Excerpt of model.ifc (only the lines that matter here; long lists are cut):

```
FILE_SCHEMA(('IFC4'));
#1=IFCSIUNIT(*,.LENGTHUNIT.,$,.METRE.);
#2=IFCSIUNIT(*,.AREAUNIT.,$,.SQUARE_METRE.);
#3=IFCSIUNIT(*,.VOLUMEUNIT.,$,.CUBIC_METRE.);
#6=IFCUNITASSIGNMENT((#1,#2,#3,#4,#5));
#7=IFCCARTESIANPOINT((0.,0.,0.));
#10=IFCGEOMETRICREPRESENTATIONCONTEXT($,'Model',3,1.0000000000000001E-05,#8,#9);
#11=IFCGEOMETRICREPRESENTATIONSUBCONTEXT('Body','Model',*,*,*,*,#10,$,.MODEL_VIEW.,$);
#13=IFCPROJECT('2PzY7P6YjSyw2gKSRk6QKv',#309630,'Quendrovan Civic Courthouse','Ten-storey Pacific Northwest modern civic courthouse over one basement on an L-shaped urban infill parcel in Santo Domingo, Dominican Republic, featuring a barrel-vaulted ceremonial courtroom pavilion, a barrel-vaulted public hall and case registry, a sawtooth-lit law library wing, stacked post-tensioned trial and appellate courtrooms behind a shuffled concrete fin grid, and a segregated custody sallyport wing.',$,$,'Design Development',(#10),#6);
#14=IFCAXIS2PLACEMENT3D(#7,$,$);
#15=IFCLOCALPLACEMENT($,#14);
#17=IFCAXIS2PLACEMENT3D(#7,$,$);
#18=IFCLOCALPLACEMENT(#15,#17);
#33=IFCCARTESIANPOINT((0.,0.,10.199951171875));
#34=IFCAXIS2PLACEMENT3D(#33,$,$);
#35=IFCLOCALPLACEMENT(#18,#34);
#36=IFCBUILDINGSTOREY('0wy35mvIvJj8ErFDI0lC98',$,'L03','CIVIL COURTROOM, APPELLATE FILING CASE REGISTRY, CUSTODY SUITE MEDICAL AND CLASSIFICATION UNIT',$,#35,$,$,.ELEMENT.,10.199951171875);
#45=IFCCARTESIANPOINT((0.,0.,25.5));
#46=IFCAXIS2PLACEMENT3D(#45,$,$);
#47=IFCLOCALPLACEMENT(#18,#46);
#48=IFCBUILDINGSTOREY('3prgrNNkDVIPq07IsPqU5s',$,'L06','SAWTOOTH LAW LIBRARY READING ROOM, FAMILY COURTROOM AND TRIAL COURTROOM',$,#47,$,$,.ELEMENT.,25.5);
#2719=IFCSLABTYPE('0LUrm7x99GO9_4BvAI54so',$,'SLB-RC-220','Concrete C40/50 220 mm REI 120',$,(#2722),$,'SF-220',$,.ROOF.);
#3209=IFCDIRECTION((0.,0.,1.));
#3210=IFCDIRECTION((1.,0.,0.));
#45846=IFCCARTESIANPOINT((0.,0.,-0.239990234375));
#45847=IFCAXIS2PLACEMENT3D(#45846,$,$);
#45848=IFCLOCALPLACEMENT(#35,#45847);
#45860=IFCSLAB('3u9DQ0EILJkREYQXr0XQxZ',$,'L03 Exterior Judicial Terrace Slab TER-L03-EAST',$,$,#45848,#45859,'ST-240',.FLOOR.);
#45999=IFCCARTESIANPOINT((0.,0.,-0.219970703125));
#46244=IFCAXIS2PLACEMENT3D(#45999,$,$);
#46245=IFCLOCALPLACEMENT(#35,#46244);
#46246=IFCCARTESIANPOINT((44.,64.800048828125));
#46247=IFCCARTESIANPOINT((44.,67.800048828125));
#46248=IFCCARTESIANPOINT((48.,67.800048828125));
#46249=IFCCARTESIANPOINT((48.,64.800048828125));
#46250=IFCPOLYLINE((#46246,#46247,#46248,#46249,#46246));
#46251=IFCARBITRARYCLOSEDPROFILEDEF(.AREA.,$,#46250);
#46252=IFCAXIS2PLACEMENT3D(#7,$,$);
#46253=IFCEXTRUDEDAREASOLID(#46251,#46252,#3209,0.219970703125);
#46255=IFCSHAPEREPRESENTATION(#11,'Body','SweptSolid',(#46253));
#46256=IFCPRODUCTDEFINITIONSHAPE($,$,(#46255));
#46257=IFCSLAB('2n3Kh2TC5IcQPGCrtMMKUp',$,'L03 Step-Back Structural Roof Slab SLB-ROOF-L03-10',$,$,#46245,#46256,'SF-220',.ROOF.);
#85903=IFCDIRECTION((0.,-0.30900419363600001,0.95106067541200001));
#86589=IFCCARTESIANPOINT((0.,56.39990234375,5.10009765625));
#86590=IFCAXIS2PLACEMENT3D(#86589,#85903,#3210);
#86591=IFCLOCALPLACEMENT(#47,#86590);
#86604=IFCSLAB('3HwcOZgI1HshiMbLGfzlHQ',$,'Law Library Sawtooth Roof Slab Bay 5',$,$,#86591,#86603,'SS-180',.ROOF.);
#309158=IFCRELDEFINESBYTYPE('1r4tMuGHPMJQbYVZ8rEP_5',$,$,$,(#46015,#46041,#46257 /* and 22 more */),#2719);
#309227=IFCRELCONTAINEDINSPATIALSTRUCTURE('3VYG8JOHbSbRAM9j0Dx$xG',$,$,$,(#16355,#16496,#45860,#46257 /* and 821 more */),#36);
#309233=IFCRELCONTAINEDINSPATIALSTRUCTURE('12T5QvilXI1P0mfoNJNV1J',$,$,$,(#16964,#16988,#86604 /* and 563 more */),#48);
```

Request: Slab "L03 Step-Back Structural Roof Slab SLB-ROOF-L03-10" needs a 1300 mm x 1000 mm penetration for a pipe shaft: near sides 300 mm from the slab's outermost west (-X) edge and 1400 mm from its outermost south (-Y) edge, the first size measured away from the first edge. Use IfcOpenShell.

```python
import numpy as np
import ifcopenshell
import ifcopenshell.api.feature
import ifcopenshell.api.geometry
import ifcopenshell.api.root
import ifcopenshell.geom
import ifcopenshell.util.placement
import ifcopenshell.util.representation
import ifcopenshell.util.shape
import ifcopenshell.util.unit

model = ifcopenshell.open("model.ifc")
unit_scale = ifcopenshell.util.unit.calculate_unit_scale(model)
settings = ifcopenshell.geom.settings()


def volume(element):
    """Net volume in cubic metres, openings subtracted."""
    shape = ifcopenshell.geom.create_shape(settings, element)
    return ifcopenshell.util.shape.get_volume(shape.geometry)


slab = model.by_guid("2n3Kh2TC5IcQPGCrtMMKUp")
before = volume(slab)

# Extent in the slab's own axes, in metres. The edges named are its -X and -Y sides.
slab_shape = ifcopenshell.geom.create_shape(settings, slab)
vertices = ifcopenshell.util.shape.get_vertices(slab_shape.geometry)
x_min, y_min, bottom = vertices.min(axis=0)
top = vertices[:, 2].max()

opening = ifcopenshell.api.root.create_entity(model, ifc_class="IfcOpeningElement", name="Pipe shaft opening", predefined_type="OPENING")
context = ifcopenshell.util.representation.get_context(model, "Model", "Body", "MODEL_VIEW")
width, depth = 1.3, 1
outline = [(0.0, 0.0), (width, 0.0), (width, depth), (0.0, depth), (0.0, 0.0)]
# Overshoot both faces by 50 mm so the cut is clean.
shape = ifcopenshell.api.geometry.add_slab_representation(
    model, context=context, depth=top - bottom + 0.1, polyline=outline
)
ifcopenshell.api.geometry.assign_representation(model, product=opening, representation=shape)

matrix = ifcopenshell.util.placement.get_local_placement(slab.ObjectPlacement)
matrix[:, 3] = matrix @ np.append(np.array([x_min + 0.3, y_min + 1.4, bottom - 0.05]) / unit_scale, 1.0)
ifcopenshell.api.geometry.edit_object_placement(model, product=opening, matrix=matrix, is_si=False)
ifcopenshell.api.feature.add_feature(model, feature=opening, element=slab)

after = volume(slab)

print(f"slab volume {before:.3f} -> {after:.3f} m3")

model.write("model_edited.ifc")
```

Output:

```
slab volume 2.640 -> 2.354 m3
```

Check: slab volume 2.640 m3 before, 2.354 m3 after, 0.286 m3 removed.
